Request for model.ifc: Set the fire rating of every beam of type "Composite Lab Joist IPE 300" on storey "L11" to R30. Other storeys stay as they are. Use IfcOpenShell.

First a look at what the model holds.

```python
import ifcopenshell
import ifcopenshell.util.element

model = ifcopenshell.open("model.ifc")
print(model.schema)
storey = next(s for s in model.by_type("IfcBuildingStorey") if s.Name == "L11")
beams = [e for e in ifcopenshell.util.element.get_decomposition(storey) if e.is_a("IfcBeam")]
seen = {}
for e in beams:
    element_type = ifcopenshell.util.element.get_type(e)
    key = (element_type.Name if element_type != e and element_type else None, ifcopenshell.util.element.get_pset(e, "Pset_BeamCommon", "FireRating"))
    seen[key] = seen.get(key, 0) + 1
for (name, value), count in sorted(seen.items(), key=str):
    print(count, "x", name, "|", value)
```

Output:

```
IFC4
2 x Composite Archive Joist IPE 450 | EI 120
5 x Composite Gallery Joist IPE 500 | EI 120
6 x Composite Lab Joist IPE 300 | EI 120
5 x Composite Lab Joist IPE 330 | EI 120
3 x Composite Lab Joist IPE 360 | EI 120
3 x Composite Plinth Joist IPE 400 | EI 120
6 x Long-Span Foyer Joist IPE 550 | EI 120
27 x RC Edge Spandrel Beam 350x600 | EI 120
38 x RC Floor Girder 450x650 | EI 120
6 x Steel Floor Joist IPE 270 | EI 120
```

```python
import ifcopenshell
import ifcopenshell.api.pset
import ifcopenshell.util.element

model = ifcopenshell.open("model.ifc")

storey = next(s for s in model.by_type("IfcBuildingStorey") if s.Name == "L11")
beams = [e for e in ifcopenshell.util.element.get_decomposition(storey) if e.is_a("IfcBeam")]

count = 0
for e in beams:
    element_type = ifcopenshell.util.element.get_type(e)
    if element_type in (None, e) or element_type.Name != "Composite Lab Joist IPE 300":
        continue
    # add_pset returns the element's existing set when there is one.
    pset = ifcopenshell.api.pset.add_pset(model, product=e, name="Pset_BeamCommon")
    ifcopenshell.api.pset.edit_pset(model, pset=pset, properties={"FireRating": "R30"})
    count += 1

print(count, "beams updated")

model.write("model_edited.ifc")
```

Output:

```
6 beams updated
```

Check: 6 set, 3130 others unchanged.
